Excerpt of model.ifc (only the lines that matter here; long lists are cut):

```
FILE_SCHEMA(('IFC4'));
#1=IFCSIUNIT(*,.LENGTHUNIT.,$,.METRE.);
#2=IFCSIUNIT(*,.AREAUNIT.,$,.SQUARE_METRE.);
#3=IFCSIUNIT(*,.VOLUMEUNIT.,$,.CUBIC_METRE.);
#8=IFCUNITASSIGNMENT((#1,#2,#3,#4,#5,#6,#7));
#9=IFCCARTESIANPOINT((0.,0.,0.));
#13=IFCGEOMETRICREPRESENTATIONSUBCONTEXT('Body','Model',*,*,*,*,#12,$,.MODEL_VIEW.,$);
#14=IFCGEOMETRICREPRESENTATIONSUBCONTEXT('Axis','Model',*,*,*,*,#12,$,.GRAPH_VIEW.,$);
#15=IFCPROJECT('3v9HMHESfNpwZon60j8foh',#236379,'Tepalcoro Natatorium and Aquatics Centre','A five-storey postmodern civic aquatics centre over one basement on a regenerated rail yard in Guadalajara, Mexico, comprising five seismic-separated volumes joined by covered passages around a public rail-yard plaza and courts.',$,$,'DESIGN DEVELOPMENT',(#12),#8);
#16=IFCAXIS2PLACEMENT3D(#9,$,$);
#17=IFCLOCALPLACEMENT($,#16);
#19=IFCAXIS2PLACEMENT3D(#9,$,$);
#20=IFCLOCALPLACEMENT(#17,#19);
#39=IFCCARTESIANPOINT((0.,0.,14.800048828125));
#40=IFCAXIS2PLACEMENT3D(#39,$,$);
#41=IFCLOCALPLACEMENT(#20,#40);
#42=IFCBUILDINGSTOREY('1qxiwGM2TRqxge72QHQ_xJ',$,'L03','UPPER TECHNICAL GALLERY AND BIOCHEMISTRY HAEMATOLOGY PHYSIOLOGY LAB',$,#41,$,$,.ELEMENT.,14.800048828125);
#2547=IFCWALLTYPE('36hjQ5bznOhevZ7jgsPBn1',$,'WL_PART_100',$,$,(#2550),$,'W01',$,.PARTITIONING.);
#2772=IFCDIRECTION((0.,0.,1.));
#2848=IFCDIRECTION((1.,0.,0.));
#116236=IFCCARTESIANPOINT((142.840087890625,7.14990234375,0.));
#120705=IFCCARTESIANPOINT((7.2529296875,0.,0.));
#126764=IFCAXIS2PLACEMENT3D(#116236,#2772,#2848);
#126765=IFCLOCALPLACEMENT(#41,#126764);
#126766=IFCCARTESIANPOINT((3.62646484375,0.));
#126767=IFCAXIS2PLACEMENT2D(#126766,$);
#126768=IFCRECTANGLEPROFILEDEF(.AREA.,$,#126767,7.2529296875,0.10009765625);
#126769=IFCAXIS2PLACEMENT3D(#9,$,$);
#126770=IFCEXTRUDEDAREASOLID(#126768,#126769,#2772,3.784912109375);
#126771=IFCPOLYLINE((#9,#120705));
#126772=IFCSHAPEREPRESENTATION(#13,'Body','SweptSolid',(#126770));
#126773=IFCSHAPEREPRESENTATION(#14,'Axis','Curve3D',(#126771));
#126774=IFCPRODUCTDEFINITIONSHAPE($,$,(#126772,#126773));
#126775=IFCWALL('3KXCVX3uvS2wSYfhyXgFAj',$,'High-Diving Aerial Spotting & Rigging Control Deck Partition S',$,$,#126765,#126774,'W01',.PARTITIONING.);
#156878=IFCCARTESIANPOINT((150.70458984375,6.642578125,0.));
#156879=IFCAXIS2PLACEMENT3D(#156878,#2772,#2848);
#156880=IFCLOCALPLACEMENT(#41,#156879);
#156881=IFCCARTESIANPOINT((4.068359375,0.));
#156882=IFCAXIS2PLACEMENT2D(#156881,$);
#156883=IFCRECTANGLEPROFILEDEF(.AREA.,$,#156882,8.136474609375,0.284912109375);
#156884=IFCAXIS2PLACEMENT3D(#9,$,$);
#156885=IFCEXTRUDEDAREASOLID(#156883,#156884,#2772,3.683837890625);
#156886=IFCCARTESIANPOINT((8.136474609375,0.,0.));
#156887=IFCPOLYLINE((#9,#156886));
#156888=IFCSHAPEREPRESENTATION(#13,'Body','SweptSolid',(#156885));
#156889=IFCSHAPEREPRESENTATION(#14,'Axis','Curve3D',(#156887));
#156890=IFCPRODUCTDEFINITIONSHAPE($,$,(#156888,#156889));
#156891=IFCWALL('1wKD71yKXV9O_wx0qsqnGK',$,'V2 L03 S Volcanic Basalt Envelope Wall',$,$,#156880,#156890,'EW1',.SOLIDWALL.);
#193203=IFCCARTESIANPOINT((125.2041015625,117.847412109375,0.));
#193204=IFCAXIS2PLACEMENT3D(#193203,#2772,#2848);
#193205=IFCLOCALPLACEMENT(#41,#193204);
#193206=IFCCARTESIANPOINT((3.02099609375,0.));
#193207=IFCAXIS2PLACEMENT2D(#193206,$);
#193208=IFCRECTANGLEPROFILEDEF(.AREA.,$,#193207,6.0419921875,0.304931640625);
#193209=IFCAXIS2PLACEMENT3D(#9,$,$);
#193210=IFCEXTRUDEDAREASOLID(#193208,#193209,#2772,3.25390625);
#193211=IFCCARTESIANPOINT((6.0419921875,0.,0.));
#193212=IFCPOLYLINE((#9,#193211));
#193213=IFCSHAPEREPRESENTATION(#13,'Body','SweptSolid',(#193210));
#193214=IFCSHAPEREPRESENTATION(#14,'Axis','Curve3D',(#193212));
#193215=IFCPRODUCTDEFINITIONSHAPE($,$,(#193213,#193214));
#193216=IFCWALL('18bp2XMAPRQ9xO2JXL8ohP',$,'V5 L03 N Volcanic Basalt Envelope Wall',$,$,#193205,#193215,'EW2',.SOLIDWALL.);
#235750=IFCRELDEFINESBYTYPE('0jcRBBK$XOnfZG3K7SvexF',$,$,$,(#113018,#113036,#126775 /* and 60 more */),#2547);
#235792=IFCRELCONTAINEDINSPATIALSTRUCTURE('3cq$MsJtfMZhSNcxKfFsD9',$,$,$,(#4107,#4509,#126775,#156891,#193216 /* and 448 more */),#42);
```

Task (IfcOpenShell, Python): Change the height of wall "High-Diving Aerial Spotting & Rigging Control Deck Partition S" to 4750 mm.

```python
import ifcopenshell
import ifcopenshell.geom
import ifcopenshell.util.representation
import ifcopenshell.util.shape
import ifcopenshell.util.unit

model = ifcopenshell.open("model.ifc")
unit_scale = ifcopenshell.util.unit.calculate_unit_scale(model)
settings = ifcopenshell.geom.settings()


def volume(element):
    """Net volume in cubic metres, openings subtracted."""
    shape = ifcopenshell.geom.create_shape(settings, element)
    return ifcopenshell.util.shape.get_volume(shape.geometry)


wall = model.by_id(126775)
before = volume(wall)

body = ifcopenshell.util.representation.get_representation(wall, "Model", "Body")
solid = body.Items[0]
old_height = solid.Depth
solid.Depth = 4.75 / unit_scale
after = volume(wall)

print(f"height {old_height:g} -> {solid.Depth:g}, volume {before:.3f} -> {after:.3f} m3")

model.write("model-out.ifc")
```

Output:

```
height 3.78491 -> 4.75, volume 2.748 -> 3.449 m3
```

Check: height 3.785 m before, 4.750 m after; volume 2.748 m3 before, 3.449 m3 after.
